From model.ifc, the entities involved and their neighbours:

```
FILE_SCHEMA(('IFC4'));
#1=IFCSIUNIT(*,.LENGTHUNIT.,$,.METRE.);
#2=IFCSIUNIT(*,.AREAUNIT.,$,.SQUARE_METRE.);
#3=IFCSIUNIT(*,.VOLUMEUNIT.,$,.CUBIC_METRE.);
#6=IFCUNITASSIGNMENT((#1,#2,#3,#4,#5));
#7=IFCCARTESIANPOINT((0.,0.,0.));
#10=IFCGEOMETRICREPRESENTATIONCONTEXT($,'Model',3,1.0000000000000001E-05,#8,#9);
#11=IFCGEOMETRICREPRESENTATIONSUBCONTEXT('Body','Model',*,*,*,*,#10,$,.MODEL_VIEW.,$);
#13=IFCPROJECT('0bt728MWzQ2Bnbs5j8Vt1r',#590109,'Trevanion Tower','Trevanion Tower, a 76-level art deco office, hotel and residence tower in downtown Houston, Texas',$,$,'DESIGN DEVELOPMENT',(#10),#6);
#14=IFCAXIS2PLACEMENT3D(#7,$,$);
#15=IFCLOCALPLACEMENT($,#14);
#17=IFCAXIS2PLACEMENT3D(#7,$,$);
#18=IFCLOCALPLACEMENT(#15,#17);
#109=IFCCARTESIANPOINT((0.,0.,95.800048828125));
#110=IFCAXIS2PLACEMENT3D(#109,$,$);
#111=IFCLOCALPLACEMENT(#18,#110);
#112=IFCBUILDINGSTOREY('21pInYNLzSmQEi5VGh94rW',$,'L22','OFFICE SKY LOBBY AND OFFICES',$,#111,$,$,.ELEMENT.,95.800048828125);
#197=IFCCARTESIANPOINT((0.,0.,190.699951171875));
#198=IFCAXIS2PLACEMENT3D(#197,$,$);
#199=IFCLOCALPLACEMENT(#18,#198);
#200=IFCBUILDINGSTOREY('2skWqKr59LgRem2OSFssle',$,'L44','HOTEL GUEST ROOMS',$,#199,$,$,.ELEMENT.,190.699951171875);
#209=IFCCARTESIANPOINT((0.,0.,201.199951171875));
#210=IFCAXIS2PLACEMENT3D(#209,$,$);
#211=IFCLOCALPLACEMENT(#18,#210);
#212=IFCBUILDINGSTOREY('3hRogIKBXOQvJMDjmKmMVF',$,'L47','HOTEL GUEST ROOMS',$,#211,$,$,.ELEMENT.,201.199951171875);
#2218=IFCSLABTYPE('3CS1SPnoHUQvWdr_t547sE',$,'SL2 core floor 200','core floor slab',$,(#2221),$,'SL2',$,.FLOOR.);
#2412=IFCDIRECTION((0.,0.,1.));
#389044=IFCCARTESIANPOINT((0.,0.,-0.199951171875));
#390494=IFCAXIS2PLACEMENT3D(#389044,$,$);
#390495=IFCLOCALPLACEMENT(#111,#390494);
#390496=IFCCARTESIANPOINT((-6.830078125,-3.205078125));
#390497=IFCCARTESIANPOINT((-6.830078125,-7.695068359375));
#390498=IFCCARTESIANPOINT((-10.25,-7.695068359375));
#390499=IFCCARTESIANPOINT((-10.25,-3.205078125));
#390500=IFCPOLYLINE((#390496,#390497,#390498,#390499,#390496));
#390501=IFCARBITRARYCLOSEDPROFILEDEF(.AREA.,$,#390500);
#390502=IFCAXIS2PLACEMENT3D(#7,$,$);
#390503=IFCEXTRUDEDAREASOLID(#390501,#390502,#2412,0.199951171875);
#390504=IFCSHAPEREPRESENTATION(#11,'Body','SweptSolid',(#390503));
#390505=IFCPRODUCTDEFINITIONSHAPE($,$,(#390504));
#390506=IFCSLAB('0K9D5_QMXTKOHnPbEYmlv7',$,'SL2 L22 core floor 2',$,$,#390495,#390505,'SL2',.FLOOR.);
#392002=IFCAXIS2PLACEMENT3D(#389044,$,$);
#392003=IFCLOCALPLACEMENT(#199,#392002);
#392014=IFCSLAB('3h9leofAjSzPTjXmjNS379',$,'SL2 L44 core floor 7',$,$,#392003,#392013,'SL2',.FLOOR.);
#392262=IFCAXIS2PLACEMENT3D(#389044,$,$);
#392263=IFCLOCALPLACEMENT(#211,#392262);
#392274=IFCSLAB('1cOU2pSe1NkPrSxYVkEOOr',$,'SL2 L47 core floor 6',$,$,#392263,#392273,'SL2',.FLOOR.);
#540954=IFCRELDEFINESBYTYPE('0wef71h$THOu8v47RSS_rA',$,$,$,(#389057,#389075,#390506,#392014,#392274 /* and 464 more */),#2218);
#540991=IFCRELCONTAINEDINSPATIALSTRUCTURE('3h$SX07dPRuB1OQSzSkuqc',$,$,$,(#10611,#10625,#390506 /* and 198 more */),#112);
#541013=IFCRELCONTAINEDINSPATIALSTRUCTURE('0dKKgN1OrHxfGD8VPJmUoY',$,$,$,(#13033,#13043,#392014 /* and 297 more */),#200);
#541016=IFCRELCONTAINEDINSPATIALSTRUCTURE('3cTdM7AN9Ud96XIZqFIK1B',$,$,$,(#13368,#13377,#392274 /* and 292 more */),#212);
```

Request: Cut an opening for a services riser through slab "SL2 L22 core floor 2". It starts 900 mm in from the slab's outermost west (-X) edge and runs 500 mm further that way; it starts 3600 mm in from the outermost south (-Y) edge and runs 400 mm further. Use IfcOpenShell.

```python
import numpy as np
import ifcopenshell
import ifcopenshell.api.feature
import ifcopenshell.api.geometry
import ifcopenshell.api.root
import ifcopenshell.geom
import ifcopenshell.util.placement
import ifcopenshell.util.representation
import ifcopenshell.util.shape
import ifcopenshell.util.unit

model = ifcopenshell.open("model.ifc")
unit_scale = ifcopenshell.util.unit.calculate_unit_scale(model)
settings = ifcopenshell.geom.settings()


def volume(element):
    """Net volume in cubic metres, openings subtracted."""
    shape = ifcopenshell.geom.create_shape(settings, element)
    return ifcopenshell.util.shape.get_volume(shape.geometry)


slab = model.by_id(390506)
before = volume(slab)

# Extent in the slab's own axes, in metres. The edges named are its -X and -Y sides.
slab_shape = ifcopenshell.geom.create_shape(settings, slab)
vertices = ifcopenshell.util.shape.get_vertices(slab_shape.geometry)
x_min, y_min, bottom = vertices.min(axis=0)
top = vertices[:, 2].max()

opening = ifcopenshell.api.root.create_entity(model, ifc_class="IfcOpeningElement", name="Services riser opening", predefined_type="OPENING")
context = ifcopenshell.util.representation.get_context(model, "Model", "Body", "MODEL_VIEW")
width, depth = 0.5, 0.4
outline = [(0.0, 0.0), (width, 0.0), (width, depth), (0.0, depth), (0.0, 0.0)]
# Overshoot both faces by 50 mm so the cut is clean.
shape = ifcopenshell.api.geometry.add_slab_representation(
    model, context=context, depth=top - bottom + 0.1, polyline=outline
)
ifcopenshell.api.geometry.assign_representation(model, product=opening, representation=shape)

matrix = ifcopenshell.util.placement.get_local_placement(slab.ObjectPlacement)
matrix[:, 3] = matrix @ np.append(np.array([x_min + 0.9, y_min + 3.6, bottom - 0.05]) / unit_scale, 1.0)
ifcopenshell.api.geometry.edit_object_placement(model, product=opening, matrix=matrix, is_si=False)
ifcopenshell.api.feature.add_feature(model, feature=opening, element=slab)

after = volume(slab)

print(f"slab volume {before:.3f} -> {after:.3f} m3")

model.write("model-out.ifc")
```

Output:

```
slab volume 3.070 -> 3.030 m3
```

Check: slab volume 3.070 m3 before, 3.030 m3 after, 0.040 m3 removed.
